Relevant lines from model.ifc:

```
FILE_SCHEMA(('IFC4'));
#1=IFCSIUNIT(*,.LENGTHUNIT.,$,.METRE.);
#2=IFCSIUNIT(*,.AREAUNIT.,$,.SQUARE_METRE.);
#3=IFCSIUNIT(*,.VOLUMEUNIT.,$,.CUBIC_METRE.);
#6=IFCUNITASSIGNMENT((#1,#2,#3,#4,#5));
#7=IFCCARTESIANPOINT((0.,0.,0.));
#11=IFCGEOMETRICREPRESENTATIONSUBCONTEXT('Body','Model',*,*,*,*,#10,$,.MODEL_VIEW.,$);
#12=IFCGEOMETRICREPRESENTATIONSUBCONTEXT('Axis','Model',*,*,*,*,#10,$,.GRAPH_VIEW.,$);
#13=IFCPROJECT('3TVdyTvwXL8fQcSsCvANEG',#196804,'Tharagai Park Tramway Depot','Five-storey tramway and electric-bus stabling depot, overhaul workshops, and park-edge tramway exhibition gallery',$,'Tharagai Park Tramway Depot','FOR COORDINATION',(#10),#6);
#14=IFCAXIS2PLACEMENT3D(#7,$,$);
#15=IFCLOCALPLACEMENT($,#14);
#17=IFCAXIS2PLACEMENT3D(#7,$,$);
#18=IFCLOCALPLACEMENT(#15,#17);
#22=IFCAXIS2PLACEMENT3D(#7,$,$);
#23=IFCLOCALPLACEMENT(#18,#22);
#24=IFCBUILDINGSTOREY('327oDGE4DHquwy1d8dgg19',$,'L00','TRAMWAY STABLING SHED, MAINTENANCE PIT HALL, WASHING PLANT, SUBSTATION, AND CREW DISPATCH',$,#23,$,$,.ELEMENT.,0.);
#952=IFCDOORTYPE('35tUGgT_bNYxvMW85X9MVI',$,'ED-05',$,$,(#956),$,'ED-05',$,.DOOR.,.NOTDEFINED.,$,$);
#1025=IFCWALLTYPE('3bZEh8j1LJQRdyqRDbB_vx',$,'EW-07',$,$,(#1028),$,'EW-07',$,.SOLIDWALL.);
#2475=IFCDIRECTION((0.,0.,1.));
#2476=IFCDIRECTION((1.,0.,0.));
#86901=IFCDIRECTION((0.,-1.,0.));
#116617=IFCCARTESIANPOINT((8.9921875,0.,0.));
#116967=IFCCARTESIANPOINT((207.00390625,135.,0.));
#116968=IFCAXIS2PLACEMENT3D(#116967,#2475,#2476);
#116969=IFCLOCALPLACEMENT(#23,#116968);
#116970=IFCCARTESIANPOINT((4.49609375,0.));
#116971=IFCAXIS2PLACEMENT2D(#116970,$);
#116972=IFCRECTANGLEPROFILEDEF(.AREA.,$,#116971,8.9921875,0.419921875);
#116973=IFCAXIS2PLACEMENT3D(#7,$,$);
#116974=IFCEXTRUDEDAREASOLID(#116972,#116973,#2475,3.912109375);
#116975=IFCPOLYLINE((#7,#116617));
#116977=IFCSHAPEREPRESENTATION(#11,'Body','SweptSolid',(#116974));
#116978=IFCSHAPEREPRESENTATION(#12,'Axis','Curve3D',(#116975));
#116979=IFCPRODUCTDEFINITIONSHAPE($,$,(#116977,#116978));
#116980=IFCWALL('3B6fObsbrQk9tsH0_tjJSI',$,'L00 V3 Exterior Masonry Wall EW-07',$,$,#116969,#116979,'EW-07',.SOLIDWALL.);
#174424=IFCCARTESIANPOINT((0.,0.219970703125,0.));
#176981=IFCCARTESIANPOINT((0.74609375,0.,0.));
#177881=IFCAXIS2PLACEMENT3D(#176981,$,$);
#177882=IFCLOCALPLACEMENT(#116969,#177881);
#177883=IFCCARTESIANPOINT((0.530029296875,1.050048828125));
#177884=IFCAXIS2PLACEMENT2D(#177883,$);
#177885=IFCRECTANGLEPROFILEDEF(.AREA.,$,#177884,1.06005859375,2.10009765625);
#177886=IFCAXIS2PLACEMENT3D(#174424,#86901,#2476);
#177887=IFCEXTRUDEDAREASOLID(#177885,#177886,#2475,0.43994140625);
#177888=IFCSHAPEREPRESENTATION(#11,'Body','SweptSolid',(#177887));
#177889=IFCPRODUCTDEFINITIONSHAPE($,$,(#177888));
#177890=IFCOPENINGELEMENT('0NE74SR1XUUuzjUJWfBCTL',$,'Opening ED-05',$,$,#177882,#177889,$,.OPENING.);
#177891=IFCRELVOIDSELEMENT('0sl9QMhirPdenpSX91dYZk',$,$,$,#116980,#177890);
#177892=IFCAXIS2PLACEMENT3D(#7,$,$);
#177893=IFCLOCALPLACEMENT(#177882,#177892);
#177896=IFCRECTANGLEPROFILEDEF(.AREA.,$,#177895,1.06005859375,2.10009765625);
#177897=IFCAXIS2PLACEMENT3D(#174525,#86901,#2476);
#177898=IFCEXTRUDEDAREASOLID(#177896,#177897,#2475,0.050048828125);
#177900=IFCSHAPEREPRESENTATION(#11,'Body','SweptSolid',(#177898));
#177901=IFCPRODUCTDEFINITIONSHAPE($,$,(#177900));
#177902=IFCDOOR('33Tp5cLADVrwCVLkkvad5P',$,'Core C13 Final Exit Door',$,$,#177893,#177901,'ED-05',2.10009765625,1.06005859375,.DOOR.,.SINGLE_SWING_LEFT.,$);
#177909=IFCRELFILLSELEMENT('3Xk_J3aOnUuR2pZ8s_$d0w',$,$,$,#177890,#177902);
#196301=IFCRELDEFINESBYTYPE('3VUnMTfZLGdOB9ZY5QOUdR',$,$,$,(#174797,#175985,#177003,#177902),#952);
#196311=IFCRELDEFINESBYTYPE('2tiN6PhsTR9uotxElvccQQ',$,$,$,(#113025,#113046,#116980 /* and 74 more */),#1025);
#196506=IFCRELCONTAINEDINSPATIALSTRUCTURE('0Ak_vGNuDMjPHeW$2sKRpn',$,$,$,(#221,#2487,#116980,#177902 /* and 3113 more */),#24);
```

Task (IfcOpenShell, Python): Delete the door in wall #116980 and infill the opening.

```python
import ifcopenshell
import ifcopenshell.api.feature
import ifcopenshell.api.root
import ifcopenshell.geom
import ifcopenshell.util.shape

model = ifcopenshell.open("model.ifc")
settings = ifcopenshell.geom.settings()


def volume(element):
    """Net volume in cubic metres, openings subtracted."""
    shape = ifcopenshell.geom.create_shape(settings, element)
    return ifcopenshell.util.shape.get_volume(shape.geometry)


door = model.by_guid("33Tp5cLADVrwCVLkkvad5P")
opening = door.FillsVoids[0].RelatingOpeningElement
wall = opening.VoidsElements[0].RelatingBuildingElement
before = volume(wall)

ifcopenshell.api.root.remove_product(model, product=door)
ifcopenshell.api.feature.remove_feature(model, feature=opening)

after = volume(wall)

print(f"wall volume {before:.3f} -> {after:.3f} m3")

model.write("model_edited.ifc")
```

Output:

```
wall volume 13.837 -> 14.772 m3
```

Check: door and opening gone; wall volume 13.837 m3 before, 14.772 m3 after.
